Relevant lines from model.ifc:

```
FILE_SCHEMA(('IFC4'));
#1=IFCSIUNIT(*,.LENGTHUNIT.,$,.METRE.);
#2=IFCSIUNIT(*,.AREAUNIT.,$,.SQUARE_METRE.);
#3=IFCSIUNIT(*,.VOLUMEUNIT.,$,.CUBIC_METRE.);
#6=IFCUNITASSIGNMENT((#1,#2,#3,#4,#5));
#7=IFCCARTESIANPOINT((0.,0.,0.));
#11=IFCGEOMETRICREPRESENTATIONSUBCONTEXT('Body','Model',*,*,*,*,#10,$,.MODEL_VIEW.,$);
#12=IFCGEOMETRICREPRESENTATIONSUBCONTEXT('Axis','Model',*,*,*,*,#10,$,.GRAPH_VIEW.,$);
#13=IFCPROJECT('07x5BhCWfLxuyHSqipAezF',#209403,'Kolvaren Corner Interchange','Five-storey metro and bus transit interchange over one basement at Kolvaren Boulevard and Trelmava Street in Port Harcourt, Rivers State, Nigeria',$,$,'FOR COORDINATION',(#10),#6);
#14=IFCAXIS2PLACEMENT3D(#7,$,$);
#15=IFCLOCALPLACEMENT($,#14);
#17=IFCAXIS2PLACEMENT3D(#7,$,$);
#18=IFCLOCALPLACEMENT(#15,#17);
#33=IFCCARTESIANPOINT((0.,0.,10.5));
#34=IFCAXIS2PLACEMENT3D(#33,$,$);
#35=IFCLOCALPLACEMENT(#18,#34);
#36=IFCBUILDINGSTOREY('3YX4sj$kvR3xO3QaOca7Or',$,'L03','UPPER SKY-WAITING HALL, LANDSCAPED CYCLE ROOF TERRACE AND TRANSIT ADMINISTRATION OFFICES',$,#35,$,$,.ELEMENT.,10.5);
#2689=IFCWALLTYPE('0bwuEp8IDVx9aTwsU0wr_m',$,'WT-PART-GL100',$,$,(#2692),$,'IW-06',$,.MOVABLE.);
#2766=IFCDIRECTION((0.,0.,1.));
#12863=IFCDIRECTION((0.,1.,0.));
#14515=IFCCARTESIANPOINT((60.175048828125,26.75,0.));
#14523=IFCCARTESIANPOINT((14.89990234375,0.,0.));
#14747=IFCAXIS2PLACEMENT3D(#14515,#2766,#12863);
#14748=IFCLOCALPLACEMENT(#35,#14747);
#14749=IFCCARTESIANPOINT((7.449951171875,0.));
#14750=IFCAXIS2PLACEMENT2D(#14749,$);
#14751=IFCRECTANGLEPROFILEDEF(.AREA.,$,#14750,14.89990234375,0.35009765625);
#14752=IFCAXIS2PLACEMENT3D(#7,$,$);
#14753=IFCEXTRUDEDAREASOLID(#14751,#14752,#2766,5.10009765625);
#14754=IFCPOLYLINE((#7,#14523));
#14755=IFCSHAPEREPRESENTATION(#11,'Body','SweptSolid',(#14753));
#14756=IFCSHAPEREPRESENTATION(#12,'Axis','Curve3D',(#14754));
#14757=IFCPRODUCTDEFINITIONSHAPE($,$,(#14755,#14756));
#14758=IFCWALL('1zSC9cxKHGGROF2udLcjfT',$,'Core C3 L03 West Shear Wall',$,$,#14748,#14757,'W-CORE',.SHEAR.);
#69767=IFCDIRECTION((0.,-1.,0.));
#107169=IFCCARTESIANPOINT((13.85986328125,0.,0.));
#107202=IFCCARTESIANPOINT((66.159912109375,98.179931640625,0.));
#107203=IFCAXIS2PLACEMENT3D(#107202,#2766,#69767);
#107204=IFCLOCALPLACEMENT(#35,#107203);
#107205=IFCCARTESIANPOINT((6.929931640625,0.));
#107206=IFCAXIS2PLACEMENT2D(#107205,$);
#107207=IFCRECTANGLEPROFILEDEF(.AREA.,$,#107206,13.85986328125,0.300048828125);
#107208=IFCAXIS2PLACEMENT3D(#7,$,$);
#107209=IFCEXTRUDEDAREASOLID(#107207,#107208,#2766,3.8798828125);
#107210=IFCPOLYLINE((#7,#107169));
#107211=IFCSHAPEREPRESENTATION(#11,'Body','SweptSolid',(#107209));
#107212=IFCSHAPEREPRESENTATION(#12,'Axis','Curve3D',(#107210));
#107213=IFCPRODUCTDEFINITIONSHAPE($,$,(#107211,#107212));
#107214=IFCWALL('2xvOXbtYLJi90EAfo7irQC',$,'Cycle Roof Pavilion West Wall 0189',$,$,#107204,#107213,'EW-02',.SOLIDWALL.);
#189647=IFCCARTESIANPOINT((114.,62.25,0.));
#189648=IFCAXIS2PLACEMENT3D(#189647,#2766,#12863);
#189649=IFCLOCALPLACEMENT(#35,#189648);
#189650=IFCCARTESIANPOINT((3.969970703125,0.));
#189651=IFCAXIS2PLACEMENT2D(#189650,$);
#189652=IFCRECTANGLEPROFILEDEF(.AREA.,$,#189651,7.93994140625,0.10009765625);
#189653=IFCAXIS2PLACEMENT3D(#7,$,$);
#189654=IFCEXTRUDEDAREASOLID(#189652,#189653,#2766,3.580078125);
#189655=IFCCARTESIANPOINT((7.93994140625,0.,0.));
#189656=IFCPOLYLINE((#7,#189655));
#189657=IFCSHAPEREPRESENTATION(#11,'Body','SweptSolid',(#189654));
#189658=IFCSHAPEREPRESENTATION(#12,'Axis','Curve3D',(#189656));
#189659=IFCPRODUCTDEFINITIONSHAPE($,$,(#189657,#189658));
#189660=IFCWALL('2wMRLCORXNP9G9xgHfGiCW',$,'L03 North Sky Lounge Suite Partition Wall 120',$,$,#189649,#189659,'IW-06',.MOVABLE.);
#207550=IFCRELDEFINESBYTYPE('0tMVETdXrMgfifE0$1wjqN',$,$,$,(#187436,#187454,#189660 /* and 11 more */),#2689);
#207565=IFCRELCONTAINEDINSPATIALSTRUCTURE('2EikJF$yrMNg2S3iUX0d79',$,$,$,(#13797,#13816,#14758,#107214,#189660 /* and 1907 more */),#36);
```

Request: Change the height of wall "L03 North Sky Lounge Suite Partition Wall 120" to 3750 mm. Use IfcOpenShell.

```python
import ifcopenshell
import ifcopenshell.geom
import ifcopenshell.util.representation
import ifcopenshell.util.shape
import ifcopenshell.util.unit

model = ifcopenshell.open("model.ifc")
unit_scale = ifcopenshell.util.unit.calculate_unit_scale(model)
settings = ifcopenshell.geom.settings()


def volume(element):
    """Net volume in cubic metres, openings subtracted."""
    shape = ifcopenshell.geom.create_shape(settings, element)
    return ifcopenshell.util.shape.get_volume(shape.geometry)


wall = model.by_id(189660)
before = volume(wall)

body = ifcopenshell.util.representation.get_representation(wall, "Model", "Body")
solid = body.Items[0]
old_height = solid.Depth
solid.Depth = 3.75 / unit_scale
after = volume(wall)

print(f"height {old_height:g} -> {solid.Depth:g}, volume {before:.3f} -> {after:.3f} m3")

model.write("model_v2.ifc")
```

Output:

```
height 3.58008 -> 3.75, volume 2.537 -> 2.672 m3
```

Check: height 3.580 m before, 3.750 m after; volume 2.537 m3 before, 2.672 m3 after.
